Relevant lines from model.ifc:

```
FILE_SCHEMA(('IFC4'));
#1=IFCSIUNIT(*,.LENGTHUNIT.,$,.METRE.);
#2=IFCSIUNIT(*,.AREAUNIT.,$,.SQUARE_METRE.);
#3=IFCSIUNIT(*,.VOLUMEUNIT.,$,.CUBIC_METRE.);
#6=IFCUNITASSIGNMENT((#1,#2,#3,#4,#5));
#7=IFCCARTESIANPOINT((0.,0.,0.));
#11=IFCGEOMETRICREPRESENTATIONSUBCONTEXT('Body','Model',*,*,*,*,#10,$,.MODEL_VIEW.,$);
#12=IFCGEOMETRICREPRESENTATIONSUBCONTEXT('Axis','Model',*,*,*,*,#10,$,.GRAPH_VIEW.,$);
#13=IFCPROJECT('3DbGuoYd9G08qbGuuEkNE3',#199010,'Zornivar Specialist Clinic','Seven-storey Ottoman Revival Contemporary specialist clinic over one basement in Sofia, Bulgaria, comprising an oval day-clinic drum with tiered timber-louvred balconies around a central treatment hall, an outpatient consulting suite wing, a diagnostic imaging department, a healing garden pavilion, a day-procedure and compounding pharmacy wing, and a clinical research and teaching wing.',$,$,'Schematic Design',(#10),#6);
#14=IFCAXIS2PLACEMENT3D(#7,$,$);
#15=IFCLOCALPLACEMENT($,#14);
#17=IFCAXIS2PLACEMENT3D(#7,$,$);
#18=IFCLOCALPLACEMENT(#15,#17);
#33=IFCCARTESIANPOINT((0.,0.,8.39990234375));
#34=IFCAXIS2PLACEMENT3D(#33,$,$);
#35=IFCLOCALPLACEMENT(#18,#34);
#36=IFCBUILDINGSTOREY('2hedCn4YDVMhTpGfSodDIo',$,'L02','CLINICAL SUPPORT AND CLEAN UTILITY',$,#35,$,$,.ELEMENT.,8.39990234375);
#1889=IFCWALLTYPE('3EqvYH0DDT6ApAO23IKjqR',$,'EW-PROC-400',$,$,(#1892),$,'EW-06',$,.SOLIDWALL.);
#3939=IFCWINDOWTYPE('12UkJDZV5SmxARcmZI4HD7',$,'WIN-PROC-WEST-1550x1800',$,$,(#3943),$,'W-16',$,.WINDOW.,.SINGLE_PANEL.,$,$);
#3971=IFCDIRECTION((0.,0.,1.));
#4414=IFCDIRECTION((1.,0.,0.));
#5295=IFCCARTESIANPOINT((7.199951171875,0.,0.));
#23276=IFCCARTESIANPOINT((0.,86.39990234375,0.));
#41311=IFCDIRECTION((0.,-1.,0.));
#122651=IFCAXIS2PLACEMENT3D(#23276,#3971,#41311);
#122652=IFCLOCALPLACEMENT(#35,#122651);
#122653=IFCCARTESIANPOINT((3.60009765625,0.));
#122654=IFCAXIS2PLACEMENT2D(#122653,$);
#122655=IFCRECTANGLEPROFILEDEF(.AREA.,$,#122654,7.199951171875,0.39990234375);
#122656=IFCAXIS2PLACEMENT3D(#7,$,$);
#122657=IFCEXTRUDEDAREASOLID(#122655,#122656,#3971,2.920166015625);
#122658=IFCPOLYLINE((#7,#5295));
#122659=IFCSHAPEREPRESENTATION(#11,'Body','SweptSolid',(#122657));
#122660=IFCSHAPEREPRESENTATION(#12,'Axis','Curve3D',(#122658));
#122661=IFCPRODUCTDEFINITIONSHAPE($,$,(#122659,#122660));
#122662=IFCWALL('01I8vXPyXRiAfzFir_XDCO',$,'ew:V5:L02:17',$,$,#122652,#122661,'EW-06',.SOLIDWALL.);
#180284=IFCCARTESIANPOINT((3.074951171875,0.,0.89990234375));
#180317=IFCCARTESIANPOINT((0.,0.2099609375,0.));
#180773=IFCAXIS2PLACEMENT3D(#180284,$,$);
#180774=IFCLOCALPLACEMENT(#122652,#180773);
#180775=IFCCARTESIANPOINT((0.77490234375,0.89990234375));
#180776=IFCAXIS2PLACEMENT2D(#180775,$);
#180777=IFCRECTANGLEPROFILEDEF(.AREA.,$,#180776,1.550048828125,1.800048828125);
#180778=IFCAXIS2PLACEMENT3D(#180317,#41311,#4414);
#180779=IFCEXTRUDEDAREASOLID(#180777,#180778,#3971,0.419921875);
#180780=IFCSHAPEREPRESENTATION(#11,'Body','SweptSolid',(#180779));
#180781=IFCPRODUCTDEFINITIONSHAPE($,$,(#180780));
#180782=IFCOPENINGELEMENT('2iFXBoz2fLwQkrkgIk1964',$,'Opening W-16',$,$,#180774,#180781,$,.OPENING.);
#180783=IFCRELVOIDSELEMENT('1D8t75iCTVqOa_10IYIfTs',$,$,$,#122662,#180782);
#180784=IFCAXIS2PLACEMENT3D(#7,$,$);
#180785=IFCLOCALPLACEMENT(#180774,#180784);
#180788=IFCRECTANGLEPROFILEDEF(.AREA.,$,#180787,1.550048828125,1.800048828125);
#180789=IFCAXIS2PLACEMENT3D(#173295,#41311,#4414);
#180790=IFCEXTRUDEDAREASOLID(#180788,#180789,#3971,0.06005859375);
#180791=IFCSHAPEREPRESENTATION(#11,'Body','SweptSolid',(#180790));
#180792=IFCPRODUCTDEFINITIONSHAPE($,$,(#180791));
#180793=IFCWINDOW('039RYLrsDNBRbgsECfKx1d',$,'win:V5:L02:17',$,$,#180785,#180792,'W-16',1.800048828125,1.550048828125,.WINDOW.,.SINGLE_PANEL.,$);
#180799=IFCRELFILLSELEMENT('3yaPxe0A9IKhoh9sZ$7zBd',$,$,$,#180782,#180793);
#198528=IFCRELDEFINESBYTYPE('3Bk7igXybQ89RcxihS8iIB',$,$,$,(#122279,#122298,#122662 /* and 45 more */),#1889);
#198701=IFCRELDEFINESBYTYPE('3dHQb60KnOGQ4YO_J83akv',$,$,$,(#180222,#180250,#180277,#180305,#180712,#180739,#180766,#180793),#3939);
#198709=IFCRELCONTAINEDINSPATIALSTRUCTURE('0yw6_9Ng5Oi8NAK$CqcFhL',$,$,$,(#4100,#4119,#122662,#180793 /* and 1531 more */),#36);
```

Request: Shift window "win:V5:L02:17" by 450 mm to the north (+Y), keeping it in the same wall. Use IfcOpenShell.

```python
import ifcopenshell
import ifcopenshell.api.geometry
import ifcopenshell.util.placement

model = ifcopenshell.open("model.ifc")

window = model.by_guid("039RYLrsDNBRbgsECfKx1d")
opening = window.FillsVoids[0].RelatingOpeningElement
wall = opening.VoidsElements[0].RelatingBuildingElement

wall_matrix = ifcopenshell.util.placement.get_local_placement(wall.ObjectPlacement)
shift = wall_matrix[:3, 0] * -0.45
before = ifcopenshell.util.placement.get_local_placement(window.ObjectPlacement)[:3, 3].copy()

# The window is placed relative to its opening, so it follows when the opening moves.
matrix = ifcopenshell.util.placement.get_local_placement(opening.ObjectPlacement)
matrix[:3, 3] += shift
ifcopenshell.api.geometry.edit_object_placement(
    model, product=opening, matrix=matrix, is_si=False, should_transform_children=True
)

after = ifcopenshell.util.placement.get_local_placement(window.ObjectPlacement)[:3, 3]
print("window moved by", (after - before).round(3) + 0.0)

model.write("model-out.ifc")
```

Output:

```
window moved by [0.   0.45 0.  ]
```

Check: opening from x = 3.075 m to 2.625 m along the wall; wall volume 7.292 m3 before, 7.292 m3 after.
